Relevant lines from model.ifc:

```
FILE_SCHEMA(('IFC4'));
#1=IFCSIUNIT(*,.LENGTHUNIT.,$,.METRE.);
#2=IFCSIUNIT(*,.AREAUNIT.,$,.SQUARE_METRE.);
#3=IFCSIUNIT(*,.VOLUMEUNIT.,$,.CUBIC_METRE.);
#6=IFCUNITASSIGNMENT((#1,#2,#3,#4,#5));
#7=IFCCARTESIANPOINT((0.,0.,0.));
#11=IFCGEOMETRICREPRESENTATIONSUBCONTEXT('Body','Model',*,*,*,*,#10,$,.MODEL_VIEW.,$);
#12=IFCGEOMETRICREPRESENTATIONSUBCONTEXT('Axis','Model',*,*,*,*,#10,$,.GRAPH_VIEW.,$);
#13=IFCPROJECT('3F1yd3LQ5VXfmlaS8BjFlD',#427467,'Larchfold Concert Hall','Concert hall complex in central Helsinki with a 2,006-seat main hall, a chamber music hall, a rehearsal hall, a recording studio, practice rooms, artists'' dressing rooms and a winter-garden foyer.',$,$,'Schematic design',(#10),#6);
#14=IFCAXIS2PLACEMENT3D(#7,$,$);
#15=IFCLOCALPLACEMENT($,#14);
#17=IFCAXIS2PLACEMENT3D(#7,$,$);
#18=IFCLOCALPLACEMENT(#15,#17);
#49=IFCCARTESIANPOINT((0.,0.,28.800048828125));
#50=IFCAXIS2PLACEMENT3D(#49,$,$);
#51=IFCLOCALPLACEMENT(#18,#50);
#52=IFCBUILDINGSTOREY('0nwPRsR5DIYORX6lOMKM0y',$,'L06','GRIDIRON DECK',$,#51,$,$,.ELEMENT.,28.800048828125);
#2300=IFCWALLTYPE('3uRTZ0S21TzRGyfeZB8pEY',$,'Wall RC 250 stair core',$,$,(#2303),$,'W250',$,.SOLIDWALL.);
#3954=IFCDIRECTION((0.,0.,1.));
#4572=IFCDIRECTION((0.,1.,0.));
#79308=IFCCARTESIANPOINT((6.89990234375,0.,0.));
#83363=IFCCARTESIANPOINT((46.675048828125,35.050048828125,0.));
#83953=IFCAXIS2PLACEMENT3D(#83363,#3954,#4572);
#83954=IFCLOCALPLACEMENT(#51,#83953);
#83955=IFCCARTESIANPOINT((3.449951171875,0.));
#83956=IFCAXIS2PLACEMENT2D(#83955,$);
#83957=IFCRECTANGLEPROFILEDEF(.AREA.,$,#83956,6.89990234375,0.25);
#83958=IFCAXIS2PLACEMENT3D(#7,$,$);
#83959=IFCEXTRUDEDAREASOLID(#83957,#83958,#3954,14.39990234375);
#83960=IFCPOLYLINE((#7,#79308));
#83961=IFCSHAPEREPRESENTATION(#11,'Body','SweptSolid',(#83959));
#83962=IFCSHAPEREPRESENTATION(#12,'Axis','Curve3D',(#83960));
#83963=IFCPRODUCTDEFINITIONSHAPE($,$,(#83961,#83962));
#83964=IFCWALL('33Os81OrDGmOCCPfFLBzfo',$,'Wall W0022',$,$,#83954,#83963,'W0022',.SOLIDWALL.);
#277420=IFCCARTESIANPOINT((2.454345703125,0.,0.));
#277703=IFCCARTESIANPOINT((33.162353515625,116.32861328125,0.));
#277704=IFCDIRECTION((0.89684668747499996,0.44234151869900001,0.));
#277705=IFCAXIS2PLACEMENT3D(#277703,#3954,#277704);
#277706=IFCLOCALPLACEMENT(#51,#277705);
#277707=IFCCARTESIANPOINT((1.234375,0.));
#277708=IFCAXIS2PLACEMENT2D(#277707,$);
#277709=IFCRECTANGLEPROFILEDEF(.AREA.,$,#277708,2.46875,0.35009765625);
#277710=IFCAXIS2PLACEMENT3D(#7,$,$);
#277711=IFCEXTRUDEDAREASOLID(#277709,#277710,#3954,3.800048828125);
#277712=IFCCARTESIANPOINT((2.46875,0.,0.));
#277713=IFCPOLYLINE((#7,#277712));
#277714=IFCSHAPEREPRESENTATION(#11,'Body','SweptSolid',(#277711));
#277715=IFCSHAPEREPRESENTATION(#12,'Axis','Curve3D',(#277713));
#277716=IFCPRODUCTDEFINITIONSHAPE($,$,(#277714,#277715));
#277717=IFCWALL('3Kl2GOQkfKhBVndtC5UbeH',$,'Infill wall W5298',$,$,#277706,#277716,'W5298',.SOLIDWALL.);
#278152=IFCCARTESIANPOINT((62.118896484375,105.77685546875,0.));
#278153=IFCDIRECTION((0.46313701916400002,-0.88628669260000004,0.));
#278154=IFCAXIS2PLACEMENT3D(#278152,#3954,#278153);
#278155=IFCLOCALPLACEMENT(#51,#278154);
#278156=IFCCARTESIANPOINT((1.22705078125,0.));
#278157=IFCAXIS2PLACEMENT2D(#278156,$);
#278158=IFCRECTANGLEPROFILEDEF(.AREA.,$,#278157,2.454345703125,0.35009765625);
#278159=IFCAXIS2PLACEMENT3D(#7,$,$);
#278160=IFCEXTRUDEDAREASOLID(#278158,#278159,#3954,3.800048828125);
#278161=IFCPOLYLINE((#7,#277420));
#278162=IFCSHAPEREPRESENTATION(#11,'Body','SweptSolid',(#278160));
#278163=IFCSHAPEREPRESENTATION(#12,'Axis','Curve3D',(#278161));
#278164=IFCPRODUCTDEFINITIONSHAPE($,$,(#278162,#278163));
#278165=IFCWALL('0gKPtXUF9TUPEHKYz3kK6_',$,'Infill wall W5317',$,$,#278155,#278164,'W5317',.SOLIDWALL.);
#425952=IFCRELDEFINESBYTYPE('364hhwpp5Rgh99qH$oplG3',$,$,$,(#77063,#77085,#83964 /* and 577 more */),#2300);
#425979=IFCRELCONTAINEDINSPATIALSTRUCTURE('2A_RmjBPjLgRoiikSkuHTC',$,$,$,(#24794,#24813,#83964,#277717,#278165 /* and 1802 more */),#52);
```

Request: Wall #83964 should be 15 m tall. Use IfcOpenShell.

```python
import ifcopenshell
import ifcopenshell.geom
import ifcopenshell.util.representation
import ifcopenshell.util.shape
import ifcopenshell.util.unit

model = ifcopenshell.open("model.ifc")
unit_scale = ifcopenshell.util.unit.calculate_unit_scale(model)
settings = ifcopenshell.geom.settings()


def volume(element):
    """Net volume in cubic metres, openings subtracted."""
    shape = ifcopenshell.geom.create_shape(settings, element)
    return ifcopenshell.util.shape.get_volume(shape.geometry)


wall = model.by_id(83964)
before = volume(wall)

body = ifcopenshell.util.representation.get_representation(wall, "Model", "Body")
solid = body.Items[0]
old_height = solid.Depth
solid.Depth = 15 / unit_scale
after = volume(wall)

print(f"height {old_height:g} -> {solid.Depth:g}, volume {before:.3f} -> {after:.3f} m3")

model.write("model_v2.ifc")
```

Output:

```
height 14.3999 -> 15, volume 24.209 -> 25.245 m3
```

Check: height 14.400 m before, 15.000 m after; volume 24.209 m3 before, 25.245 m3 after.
